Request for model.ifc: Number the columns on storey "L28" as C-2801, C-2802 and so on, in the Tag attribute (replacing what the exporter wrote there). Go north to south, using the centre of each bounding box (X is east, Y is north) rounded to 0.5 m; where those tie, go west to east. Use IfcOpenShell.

First a look at what the model holds.

```python
import ifcopenshell
import ifcopenshell.util.element
import ifcopenshell.util.placement

model = ifcopenshell.open("model.ifc")
print(model.schema)
storey = next(s for s in model.by_type("IfcBuildingStorey") if s.Name == "L28")
columns = [e for e in ifcopenshell.util.element.get_decomposition(storey) if e.is_a("IfcColumn")]
for e in sorted(columns, key=lambda e: e.id()):
    origin = ifcopenshell.util.placement.get_local_placement(e.ObjectPlacement)[:3, 3]
    print(e.id(), e.Tag, e.Name, origin.round(2) + 0.0, sep=" | ")
```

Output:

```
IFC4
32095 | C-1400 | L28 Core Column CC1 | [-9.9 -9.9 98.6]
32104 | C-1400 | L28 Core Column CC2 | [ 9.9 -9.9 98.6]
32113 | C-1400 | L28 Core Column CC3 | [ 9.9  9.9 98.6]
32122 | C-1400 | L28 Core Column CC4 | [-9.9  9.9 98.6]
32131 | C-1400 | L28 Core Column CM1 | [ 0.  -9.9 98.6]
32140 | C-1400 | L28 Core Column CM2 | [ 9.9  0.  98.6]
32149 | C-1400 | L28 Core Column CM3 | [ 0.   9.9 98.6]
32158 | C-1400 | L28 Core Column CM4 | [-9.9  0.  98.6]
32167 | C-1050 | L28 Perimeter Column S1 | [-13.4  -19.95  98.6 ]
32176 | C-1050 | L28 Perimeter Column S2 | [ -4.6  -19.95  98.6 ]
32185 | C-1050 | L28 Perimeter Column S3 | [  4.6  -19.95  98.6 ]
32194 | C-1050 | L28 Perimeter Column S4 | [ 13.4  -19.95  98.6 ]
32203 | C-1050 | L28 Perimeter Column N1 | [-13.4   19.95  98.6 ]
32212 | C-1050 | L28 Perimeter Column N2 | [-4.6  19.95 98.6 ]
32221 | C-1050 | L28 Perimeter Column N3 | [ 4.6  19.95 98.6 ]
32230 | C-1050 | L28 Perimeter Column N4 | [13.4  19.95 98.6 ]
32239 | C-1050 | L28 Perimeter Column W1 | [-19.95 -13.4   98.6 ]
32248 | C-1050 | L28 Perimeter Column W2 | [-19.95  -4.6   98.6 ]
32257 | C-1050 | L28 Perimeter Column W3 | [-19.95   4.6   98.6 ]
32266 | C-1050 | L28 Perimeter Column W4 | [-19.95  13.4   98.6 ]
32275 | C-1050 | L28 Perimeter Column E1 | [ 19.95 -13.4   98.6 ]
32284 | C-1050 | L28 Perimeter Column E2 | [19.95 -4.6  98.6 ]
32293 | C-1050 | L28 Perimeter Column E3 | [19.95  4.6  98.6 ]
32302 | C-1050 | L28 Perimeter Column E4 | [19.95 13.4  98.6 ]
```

```python
import ifcopenshell
import ifcopenshell.geom
import ifcopenshell.util.element
import ifcopenshell.util.shape

model = ifcopenshell.open("model.ifc")
settings = ifcopenshell.geom.settings()
settings.set("use-world-coords", True)


def centre(element):
    shape = ifcopenshell.geom.create_shape(settings, element)
    return ifcopenshell.util.shape.get_bbox_centroid(shape.geometry)


storey = next(s for s in model.by_type("IfcBuildingStorey") if s.Name == "L28")
columns = [e for e in ifcopenshell.util.element.get_decomposition(storey) if e.is_a("IfcColumn")]

# Insertion points can sit at a corner or the storey origin, so sort by the geometry (in metres).
centres = {e: centre(e) for e in columns}
columns.sort(key=lambda e: (-round(centres[e][1] / 0.5), centres[e][0]))

for i, e in enumerate(columns, start=1):
    number = f"C-28{i:02d}"
    e.Tag = number
    print(e.id(), number)

model.write("model_updated.ifc")
```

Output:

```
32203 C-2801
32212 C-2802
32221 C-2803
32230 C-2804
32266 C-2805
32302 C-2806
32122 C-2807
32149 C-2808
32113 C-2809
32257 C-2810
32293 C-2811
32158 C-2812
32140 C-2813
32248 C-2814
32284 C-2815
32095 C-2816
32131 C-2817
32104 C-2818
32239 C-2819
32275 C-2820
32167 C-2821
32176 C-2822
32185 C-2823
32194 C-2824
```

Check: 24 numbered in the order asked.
